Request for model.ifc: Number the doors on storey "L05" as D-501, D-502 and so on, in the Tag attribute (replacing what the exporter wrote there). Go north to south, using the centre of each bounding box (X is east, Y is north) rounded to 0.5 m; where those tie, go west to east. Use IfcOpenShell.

First a look at what the model holds.

```python
import ifcopenshell
import ifcopenshell.util.element
import ifcopenshell.util.placement

model = ifcopenshell.open("model.ifc")
print(model.schema)
storey = next(s for s in model.by_type("IfcBuildingStorey") if s.Name == "L05")
doors = [e for e in ifcopenshell.util.element.get_decomposition(storey) if e.is_a("IfcDoor")]
for e in sorted(doors, key=lambda e: e.id()):
    origin = ifcopenshell.util.placement.get_local_placement(e.ObjectPlacement)[:3, 3]
    print(e.id(), e.Tag, e.Name, origin.round(2) + 0.0, sep=" | ")
```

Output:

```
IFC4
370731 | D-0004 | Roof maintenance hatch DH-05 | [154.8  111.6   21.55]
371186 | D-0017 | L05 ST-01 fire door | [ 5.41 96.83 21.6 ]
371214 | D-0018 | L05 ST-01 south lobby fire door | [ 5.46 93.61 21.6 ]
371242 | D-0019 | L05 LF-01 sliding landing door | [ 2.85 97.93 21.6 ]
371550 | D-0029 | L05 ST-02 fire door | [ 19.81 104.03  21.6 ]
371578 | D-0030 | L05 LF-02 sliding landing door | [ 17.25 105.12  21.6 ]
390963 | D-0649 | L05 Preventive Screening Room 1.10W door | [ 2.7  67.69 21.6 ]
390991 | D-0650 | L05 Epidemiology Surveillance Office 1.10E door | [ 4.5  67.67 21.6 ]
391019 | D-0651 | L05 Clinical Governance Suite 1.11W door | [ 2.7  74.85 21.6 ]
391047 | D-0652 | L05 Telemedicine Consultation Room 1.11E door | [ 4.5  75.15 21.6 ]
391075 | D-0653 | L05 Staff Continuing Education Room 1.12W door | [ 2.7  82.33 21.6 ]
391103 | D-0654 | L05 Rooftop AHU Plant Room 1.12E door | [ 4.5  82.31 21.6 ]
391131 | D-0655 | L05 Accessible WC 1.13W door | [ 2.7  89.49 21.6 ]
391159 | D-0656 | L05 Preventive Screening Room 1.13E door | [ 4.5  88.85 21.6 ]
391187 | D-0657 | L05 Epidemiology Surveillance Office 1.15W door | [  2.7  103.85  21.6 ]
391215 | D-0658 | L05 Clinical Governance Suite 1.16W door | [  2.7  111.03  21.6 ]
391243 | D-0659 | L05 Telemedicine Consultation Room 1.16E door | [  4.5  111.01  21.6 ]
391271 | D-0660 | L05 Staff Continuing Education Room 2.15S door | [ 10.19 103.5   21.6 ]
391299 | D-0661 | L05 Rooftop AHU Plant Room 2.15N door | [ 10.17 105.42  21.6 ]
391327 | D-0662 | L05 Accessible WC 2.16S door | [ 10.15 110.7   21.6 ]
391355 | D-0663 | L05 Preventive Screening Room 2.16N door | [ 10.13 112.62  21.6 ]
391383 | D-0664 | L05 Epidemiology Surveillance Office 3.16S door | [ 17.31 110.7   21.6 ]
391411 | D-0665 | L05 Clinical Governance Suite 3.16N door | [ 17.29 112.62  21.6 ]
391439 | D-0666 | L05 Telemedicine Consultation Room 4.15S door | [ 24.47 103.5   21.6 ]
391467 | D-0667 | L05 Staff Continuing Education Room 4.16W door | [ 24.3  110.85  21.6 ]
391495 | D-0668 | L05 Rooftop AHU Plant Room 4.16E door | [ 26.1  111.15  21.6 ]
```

```python
import ifcopenshell
import ifcopenshell.geom
import ifcopenshell.util.element
import ifcopenshell.util.shape

model = ifcopenshell.open("model.ifc")
settings = ifcopenshell.geom.settings()
settings.set("use-world-coords", True)


def centre(element):
    shape = ifcopenshell.geom.create_shape(settings, element)
    return ifcopenshell.util.shape.get_bbox_centroid(shape.geometry)


storey = next(s for s in model.by_type("IfcBuildingStorey") if s.Name == "L05")
doors = [e for e in ifcopenshell.util.element.get_decomposition(storey) if e.is_a("IfcDoor")]

# Insertion points can sit at a corner or the storey origin, so sort by the geometry (in metres).
centres = {e: centre(e) for e in doors}
doors.sort(key=lambda e: (-round(centres[e][1] / 0.5), centres[e][0]))

for i, e in enumerate(doors, start=1):
    number = f"D-5{i:02d}"
    e.Tag = number
    print(e.id(), number)

model.write("model_v2.ifc")
```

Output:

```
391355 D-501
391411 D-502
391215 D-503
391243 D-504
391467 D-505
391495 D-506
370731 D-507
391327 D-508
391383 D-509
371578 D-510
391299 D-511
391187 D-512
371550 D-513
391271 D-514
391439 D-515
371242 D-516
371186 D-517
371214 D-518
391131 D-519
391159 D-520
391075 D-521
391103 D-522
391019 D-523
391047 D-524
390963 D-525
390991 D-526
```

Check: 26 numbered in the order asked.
